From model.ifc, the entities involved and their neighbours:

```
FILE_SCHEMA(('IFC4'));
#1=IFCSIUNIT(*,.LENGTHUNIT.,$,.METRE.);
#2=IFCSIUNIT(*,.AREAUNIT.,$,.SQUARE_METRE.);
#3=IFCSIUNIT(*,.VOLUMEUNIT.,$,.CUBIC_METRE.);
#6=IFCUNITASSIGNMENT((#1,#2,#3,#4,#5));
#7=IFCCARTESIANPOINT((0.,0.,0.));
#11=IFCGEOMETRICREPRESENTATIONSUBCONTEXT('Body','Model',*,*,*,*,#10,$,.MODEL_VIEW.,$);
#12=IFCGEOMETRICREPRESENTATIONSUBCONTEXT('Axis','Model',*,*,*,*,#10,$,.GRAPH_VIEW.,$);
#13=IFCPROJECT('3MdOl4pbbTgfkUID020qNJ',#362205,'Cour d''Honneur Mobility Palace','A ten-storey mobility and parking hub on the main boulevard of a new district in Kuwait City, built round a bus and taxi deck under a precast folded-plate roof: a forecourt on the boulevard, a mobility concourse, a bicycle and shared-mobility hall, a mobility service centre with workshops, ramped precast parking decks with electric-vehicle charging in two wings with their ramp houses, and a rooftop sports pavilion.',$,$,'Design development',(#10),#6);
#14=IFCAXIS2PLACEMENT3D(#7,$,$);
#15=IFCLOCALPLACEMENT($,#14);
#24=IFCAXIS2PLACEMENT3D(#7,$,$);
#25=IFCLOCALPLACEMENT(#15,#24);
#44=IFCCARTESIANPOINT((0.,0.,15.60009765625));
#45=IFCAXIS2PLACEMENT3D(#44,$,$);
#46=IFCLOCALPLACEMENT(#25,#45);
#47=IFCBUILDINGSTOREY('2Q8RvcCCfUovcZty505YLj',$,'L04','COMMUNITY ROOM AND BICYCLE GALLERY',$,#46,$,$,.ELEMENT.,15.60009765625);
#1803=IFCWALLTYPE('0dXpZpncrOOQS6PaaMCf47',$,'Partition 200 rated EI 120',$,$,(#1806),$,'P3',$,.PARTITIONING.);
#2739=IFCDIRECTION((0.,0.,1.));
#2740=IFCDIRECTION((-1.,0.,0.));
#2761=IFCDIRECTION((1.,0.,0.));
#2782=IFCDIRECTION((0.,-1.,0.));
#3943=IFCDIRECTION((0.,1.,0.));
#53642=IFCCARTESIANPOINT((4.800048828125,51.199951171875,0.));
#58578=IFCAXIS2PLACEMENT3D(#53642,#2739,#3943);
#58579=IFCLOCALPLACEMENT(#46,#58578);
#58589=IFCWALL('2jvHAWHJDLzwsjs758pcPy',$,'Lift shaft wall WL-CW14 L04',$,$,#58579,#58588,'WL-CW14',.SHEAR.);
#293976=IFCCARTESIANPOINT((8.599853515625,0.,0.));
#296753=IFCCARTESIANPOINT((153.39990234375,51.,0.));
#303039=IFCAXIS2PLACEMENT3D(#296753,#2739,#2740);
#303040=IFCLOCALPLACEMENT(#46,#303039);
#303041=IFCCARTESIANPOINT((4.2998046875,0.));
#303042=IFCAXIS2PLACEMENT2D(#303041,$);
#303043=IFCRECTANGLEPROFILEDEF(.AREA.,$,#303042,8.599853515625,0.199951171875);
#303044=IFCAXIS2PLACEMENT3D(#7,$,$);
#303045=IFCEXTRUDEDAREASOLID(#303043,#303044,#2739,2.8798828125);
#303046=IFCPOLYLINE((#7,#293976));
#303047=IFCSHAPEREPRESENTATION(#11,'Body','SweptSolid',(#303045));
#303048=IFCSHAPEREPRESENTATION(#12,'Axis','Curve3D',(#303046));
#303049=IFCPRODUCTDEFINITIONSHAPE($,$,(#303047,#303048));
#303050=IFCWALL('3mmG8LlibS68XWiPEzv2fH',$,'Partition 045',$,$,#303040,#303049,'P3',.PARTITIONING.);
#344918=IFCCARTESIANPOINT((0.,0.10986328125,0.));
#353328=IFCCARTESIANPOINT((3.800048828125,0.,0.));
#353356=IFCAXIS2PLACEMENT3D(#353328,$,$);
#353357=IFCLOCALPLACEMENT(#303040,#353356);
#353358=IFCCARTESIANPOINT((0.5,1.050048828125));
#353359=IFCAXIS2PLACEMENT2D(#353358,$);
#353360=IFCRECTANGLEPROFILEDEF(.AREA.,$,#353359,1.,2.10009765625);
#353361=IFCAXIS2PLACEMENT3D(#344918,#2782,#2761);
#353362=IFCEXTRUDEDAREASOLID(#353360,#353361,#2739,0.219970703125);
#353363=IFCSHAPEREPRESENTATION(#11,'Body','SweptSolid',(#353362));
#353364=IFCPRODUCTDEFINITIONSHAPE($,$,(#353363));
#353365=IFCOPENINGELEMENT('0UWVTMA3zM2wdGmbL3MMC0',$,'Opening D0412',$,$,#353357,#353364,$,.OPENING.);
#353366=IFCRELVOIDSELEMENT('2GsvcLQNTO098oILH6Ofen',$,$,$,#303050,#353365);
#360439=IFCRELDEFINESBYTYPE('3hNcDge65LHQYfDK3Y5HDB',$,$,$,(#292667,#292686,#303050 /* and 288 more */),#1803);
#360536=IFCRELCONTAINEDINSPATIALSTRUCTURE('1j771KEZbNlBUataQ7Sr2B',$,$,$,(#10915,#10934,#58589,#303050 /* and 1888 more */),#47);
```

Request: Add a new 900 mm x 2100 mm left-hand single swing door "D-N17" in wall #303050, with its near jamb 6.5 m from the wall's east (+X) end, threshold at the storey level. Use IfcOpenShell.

```python
import numpy as np
import ifcopenshell
import ifcopenshell.api.feature
import ifcopenshell.api.geometry
import ifcopenshell.api.root
import ifcopenshell.api.spatial
import ifcopenshell.geom
import ifcopenshell.util.element
import ifcopenshell.util.placement
import ifcopenshell.util.representation
import ifcopenshell.util.shape
import ifcopenshell.util.unit

model = ifcopenshell.open("model.ifc")
unit_scale = ifcopenshell.util.unit.calculate_unit_scale(model)
settings = ifcopenshell.geom.settings()


def volume(element):
    """Net volume in cubic metres, openings subtracted."""
    shape = ifcopenshell.geom.create_shape(settings, element)
    return ifcopenshell.util.shape.get_volume(shape.geometry)


wall = model.by_guid("3mmG8LlibS68XWiPEzv2fH")
storey = ifcopenshell.util.element.get_container(wall, ifc_class="IfcBuildingStorey")
context = ifcopenshell.util.representation.get_context(model, "Model", "Body", "MODEL_VIEW")
before = volume(wall)

width, height, from_end, sill = 0.9, 2.1, 6.5, 0.0  # metres

# The wall runs along its own X axis, and the end named is its -X end.
wall_shape = ifcopenshell.geom.create_shape(settings, wall)
x, y, z = ifcopenshell.util.shape.get_vertices(wall_shape.geometry).T
start = x.min() + from_end
face, thickness = float(y.min()), float(y.max() - y.min())
wall_matrix = ifcopenshell.util.placement.get_local_placement(wall.ObjectPlacement)
level = ifcopenshell.util.placement.get_local_placement(storey.ObjectPlacement)[2, 3]


def in_wall(x, y):
    """Placement at x, y metres in the wall's axes, at sill height."""
    matrix = wall_matrix.copy()
    matrix[:, 3] = wall_matrix @ np.array([x / unit_scale, y / unit_scale, 0.0, 1.0])
    matrix[2, 3] = level + sill / unit_scale
    return matrix


# Opening: a box that overshoots both wall faces by 50 mm.
opening = ifcopenshell.api.root.create_entity(model, ifc_class="IfcOpeningElement", predefined_type="OPENING")
box = ifcopenshell.api.geometry.add_wall_representation(
    model, context=context, length=width, height=height, thickness=thickness + 0.1
)
ifcopenshell.api.geometry.assign_representation(model, product=opening, representation=box)
ifcopenshell.api.geometry.edit_object_placement(model, product=opening, matrix=in_wall(start, face - 0.05), is_si=False)
ifcopenshell.api.feature.add_feature(model, feature=opening, element=wall)

door = ifcopenshell.api.root.create_entity(model, ifc_class="IfcDoor", name="D-N17", predefined_type="DOOR")
door.OverallWidth, door.OverallHeight = width / unit_scale, height / unit_scale
door.OperationType = "SINGLE_SWING_LEFT"
body = ifcopenshell.api.geometry.add_door_representation(
    model,
    context=context,
    overall_width=door.OverallWidth,
    overall_height=door.OverallHeight,
    operation_type="SINGLE_SWING_LEFT",
    lining_properties={"LiningDepth": thickness / unit_scale, "ThresholdDepth": thickness / unit_scale},
)
ifcopenshell.api.geometry.assign_representation(model, product=door, representation=body)
ifcopenshell.api.spatial.assign_container(model, products=[door], relating_structure=storey)
ifcopenshell.api.feature.add_filling(model, opening=opening, element=door)

# The lining spans the wall, so the door starts at the wall face.
ifcopenshell.api.geometry.edit_object_placement(model, product=door, matrix=in_wall(start, face), is_si=False)

after = volume(wall)

print(f"wall volume {before:.3f} -> {after:.3f} m3")

model.write("model_v2.ifc")
```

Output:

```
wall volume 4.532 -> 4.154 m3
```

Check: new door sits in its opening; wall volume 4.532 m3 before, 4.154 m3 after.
